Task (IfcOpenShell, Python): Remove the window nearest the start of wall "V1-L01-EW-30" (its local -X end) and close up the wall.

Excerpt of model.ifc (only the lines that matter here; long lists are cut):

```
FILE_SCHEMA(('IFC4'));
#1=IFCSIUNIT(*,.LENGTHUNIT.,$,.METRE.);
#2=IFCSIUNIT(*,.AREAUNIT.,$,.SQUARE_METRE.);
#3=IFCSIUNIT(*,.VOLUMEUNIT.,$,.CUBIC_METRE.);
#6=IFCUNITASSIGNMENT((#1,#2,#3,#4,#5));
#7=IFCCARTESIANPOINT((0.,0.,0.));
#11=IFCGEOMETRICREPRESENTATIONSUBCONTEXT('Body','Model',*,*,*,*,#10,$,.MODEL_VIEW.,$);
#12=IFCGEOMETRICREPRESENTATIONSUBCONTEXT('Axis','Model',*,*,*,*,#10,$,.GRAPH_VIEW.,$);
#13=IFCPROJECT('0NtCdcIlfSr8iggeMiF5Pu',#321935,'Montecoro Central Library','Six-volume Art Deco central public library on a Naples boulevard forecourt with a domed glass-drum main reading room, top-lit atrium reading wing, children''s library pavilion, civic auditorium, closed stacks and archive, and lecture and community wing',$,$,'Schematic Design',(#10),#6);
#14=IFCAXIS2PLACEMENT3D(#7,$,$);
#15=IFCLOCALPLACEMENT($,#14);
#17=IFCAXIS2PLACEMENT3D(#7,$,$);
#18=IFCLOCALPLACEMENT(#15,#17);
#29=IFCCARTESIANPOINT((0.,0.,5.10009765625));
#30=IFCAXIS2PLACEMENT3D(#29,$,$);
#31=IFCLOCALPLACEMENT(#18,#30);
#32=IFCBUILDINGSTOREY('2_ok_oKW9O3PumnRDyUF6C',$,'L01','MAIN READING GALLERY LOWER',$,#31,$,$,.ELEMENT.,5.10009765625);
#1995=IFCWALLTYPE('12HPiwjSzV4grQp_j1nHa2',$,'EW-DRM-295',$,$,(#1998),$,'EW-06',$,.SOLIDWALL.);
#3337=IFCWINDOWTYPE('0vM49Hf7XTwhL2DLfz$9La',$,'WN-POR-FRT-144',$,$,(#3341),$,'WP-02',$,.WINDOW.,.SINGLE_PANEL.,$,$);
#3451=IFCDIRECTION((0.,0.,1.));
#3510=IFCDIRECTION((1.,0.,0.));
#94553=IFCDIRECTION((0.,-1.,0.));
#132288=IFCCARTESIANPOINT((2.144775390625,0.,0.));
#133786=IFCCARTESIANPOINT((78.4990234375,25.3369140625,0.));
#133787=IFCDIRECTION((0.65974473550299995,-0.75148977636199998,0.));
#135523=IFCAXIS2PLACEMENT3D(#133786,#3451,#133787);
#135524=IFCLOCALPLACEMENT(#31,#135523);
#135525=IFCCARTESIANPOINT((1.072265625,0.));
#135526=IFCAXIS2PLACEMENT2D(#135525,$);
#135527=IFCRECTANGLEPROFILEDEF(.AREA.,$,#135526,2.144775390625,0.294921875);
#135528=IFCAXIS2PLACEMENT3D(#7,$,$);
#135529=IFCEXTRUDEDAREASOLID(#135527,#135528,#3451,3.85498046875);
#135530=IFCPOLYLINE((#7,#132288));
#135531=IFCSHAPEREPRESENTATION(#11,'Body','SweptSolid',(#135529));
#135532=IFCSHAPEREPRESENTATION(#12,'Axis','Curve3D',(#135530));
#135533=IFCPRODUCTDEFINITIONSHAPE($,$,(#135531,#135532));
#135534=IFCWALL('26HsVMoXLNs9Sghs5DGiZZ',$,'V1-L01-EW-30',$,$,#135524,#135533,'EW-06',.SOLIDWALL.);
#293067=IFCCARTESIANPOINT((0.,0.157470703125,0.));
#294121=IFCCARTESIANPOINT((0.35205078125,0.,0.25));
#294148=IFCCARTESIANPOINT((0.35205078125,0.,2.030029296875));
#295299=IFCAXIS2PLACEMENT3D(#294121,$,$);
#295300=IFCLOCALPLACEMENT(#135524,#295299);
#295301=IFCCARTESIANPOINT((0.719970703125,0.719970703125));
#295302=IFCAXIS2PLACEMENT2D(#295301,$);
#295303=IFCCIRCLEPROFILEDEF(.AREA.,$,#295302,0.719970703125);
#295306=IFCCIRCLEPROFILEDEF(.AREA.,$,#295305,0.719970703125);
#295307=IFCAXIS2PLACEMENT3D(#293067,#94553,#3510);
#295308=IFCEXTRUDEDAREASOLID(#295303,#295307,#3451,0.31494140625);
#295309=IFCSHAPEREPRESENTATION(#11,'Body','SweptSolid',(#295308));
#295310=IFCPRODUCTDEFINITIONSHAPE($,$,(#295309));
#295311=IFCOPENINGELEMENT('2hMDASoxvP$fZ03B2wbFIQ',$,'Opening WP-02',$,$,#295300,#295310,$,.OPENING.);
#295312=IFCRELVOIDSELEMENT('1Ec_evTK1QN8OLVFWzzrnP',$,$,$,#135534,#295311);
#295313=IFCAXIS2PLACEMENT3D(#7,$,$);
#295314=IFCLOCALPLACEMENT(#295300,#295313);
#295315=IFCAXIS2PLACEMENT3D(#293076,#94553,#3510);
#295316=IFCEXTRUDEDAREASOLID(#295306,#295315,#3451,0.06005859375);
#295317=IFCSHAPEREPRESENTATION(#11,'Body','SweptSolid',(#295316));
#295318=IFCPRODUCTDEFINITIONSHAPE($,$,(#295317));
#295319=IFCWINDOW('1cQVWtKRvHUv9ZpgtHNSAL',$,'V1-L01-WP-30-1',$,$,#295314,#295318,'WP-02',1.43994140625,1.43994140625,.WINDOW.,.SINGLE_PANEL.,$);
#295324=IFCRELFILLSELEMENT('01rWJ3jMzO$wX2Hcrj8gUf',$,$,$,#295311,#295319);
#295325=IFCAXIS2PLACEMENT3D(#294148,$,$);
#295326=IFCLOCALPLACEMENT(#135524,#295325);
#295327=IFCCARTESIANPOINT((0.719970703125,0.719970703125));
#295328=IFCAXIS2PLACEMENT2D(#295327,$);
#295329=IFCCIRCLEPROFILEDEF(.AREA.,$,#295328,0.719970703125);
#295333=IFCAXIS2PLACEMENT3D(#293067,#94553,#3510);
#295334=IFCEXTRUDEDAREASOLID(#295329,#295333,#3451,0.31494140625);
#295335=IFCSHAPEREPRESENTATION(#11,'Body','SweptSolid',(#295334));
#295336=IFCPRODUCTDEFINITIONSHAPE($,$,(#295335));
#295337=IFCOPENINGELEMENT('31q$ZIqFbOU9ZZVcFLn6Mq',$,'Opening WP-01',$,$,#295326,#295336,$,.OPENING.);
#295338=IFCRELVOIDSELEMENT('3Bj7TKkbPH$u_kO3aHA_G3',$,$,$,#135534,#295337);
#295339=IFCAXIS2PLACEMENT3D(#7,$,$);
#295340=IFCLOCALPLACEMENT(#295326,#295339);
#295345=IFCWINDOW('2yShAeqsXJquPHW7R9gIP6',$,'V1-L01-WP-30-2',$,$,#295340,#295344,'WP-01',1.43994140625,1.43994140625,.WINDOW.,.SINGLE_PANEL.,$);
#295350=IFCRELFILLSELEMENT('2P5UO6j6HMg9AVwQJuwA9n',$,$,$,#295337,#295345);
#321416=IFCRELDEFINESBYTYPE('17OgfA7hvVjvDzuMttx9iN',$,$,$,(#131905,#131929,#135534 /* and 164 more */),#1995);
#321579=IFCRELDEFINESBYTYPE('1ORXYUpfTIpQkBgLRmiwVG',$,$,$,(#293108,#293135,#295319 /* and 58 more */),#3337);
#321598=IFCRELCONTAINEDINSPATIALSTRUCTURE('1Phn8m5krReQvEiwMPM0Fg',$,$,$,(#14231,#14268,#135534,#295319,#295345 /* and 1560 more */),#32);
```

```python
import ifcopenshell
import ifcopenshell.api.feature
import ifcopenshell.api.root
import ifcopenshell.geom
import ifcopenshell.util.shape

model = ifcopenshell.open("model.ifc")
settings = ifcopenshell.geom.settings()


def volume(element):
    """Net volume in cubic metres, openings subtracted."""
    shape = ifcopenshell.geom.create_shape(settings, element)
    return ifcopenshell.util.shape.get_volume(shape.geometry)


window = model.by_id(295319)
opening = window.FillsVoids[0].RelatingOpeningElement
wall = opening.VoidsElements[0].RelatingBuildingElement
before = volume(wall)

ifcopenshell.api.root.remove_product(model, product=window)
ifcopenshell.api.feature.remove_feature(model, feature=opening)

after = volume(wall)

print(f"wall volume {before:.3f} -> {after:.3f} m3")

model.write("model_rev.ifc")
```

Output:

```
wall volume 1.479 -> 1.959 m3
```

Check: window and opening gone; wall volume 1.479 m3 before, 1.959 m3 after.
